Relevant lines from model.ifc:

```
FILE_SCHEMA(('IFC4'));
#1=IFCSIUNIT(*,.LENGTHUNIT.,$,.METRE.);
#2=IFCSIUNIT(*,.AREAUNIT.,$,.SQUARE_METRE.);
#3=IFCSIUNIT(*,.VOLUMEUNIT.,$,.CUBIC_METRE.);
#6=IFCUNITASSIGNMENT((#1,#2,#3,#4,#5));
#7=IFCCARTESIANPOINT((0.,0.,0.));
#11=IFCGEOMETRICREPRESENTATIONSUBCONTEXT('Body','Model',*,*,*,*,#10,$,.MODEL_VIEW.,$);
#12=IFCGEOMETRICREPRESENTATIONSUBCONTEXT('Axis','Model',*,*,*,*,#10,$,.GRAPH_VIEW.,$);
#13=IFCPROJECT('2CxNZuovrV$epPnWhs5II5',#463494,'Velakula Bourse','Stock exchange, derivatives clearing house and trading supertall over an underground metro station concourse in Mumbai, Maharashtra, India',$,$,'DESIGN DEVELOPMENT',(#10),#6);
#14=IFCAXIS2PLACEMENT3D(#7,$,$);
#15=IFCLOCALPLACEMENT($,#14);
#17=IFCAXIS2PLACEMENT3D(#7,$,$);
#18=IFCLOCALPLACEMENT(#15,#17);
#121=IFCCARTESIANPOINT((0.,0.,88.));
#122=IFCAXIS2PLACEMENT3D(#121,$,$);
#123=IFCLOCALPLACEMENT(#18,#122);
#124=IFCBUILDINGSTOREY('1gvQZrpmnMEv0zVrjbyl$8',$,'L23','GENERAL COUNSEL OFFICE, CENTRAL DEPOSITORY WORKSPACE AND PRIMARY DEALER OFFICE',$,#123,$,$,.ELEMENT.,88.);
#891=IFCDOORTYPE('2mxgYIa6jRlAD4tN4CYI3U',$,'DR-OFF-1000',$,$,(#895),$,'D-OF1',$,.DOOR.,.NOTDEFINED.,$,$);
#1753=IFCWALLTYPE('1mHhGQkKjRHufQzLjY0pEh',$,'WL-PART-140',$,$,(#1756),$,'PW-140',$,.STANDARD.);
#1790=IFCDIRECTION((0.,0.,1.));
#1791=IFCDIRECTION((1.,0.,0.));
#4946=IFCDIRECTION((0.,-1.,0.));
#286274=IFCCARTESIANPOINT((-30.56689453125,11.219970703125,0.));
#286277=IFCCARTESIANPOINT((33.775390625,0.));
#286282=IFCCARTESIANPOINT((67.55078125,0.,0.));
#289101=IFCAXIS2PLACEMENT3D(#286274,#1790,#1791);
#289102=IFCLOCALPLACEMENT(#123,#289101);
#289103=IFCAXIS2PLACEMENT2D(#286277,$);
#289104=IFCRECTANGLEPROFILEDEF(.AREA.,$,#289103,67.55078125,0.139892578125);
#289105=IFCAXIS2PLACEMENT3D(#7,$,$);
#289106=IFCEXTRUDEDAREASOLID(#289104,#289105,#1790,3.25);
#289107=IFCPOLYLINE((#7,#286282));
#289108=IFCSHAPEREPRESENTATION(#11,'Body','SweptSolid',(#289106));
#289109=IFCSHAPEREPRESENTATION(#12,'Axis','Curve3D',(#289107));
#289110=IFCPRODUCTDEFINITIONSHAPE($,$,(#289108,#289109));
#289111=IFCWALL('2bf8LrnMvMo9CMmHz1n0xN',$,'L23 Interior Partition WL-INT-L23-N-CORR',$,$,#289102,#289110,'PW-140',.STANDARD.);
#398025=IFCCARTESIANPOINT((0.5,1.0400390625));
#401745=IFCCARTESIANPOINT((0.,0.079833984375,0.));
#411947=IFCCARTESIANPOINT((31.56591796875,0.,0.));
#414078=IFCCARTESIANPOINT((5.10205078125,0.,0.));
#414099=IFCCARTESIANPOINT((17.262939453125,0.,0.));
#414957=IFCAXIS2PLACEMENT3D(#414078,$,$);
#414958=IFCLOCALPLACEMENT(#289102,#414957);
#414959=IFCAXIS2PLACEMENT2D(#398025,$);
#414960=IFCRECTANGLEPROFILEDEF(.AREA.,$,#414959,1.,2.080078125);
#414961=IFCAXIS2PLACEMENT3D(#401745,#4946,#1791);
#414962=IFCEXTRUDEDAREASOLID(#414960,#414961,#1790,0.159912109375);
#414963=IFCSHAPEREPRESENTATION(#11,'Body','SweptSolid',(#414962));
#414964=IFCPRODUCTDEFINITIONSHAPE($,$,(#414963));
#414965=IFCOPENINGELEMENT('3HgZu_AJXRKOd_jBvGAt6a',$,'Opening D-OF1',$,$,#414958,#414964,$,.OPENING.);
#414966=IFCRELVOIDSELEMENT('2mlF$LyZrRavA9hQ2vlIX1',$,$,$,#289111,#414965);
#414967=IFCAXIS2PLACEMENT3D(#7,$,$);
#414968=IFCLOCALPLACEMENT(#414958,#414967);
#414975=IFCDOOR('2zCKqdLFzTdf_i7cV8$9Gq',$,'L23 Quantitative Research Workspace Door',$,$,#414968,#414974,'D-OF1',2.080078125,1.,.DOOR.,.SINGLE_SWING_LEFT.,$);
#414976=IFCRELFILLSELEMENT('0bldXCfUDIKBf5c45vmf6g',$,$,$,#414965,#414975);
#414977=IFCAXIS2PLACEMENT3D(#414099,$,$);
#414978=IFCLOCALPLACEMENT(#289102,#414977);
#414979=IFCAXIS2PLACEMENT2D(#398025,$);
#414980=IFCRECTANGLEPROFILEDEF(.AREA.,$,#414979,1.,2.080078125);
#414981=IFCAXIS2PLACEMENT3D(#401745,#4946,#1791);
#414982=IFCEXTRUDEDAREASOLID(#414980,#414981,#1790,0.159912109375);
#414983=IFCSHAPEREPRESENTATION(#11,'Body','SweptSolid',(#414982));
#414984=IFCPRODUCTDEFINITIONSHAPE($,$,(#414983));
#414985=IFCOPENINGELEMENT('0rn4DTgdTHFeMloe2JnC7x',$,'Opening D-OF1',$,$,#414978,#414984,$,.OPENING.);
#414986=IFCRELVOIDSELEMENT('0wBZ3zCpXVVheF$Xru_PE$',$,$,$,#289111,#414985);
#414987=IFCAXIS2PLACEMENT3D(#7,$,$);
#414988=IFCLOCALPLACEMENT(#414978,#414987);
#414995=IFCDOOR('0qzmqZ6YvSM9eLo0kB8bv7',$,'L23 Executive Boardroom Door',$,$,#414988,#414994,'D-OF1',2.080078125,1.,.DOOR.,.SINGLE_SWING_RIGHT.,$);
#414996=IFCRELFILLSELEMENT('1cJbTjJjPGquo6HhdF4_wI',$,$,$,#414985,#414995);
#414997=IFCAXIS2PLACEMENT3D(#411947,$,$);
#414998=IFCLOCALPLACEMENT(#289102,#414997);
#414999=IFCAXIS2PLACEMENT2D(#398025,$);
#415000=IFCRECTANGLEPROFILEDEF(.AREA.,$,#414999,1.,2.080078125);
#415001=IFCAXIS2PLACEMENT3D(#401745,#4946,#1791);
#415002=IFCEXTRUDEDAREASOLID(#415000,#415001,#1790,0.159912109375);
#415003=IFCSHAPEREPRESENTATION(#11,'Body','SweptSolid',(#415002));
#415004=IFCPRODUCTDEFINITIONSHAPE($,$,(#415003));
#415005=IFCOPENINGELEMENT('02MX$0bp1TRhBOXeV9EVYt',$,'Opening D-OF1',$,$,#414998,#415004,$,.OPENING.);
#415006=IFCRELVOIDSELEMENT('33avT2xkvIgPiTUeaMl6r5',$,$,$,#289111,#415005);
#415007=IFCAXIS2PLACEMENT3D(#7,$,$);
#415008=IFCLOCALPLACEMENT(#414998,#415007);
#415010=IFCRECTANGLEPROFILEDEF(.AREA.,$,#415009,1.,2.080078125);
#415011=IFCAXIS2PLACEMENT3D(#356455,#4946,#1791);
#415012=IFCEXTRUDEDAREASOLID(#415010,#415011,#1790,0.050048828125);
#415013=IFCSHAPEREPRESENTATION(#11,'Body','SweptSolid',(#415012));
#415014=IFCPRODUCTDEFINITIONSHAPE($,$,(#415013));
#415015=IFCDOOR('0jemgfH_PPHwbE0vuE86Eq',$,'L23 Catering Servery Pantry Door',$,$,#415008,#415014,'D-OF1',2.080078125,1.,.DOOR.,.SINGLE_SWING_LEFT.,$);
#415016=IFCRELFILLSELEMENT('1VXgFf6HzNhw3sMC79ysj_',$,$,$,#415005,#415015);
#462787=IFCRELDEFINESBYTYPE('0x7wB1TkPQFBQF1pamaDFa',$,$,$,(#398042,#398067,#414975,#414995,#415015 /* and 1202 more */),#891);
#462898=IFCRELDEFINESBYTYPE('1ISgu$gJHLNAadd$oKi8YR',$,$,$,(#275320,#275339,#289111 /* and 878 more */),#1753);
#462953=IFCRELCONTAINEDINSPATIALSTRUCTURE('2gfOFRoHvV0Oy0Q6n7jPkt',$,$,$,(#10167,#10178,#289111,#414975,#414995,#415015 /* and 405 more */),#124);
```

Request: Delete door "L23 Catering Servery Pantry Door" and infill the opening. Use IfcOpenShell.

```python
import ifcopenshell
import ifcopenshell.api.feature
import ifcopenshell.api.root
import ifcopenshell.geom
import ifcopenshell.util.shape

model = ifcopenshell.open("model.ifc")
settings = ifcopenshell.geom.settings()


def volume(element):
    """Net volume in cubic metres, openings subtracted."""
    shape = ifcopenshell.geom.create_shape(settings, element)
    return ifcopenshell.util.shape.get_volume(shape.geometry)


door = model.by_id(415015)
opening = door.FillsVoids[0].RelatingOpeningElement
wall = opening.VoidsElements[0].RelatingBuildingElement
before = volume(wall)

ifcopenshell.api.root.remove_product(model, product=door)
ifcopenshell.api.feature.remove_feature(model, feature=opening)

after = volume(wall)

print(f"wall volume {before:.3f} -> {after:.3f} m3")

model.write("model-out.ifc")
```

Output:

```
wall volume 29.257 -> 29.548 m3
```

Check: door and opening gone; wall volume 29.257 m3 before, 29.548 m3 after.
